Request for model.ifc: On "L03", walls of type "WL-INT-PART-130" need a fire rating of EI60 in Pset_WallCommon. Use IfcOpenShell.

First a look at what the model holds.

```python
import ifcopenshell
import ifcopenshell.util.element

model = ifcopenshell.open("model.ifc")
print(model.schema)
storey = next(s for s in model.by_type("IfcBuildingStorey") if s.Name == "L03")
walls = [e for e in ifcopenshell.util.element.get_decomposition(storey) if e.is_a("IfcWall")]
seen = {}
for e in walls:
    element_type = ifcopenshell.util.element.get_type(e)
    key = (element_type.Name if element_type != e and element_type else None, ifcopenshell.util.element.get_pset(e, "Pset_WallCommon", "FireRating"))
    seen[key] = seen.get(key, 0) + 1
for (name, value), count in sorted(seen.items(), key=str):
    print(count, "x", name, "|", value)
```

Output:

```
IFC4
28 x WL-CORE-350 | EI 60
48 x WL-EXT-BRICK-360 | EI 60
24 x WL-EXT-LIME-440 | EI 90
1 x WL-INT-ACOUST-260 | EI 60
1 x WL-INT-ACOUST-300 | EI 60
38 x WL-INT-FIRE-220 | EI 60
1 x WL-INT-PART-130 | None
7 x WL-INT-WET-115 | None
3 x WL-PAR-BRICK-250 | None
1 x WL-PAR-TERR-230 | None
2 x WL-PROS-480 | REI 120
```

```python
import ifcopenshell
import ifcopenshell.api.pset
import ifcopenshell.util.element

model = ifcopenshell.open("model.ifc")

storey = next(s for s in model.by_type("IfcBuildingStorey") if s.Name == "L03")
walls = [e for e in ifcopenshell.util.element.get_decomposition(storey) if e.is_a("IfcWall")]

count = 0
for e in walls:
    element_type = ifcopenshell.util.element.get_type(e)
    if element_type in (None, e) or element_type.Name != "WL-INT-PART-130":
        continue
    # add_pset returns the element's existing set when there is one.
    pset = ifcopenshell.api.pset.add_pset(model, product=e, name="Pset_WallCommon")
    ifcopenshell.api.pset.edit_pset(model, pset=pset, properties={"FireRating": "EI60"})
    count += 1

print(count, "walls updated")

model.write("model-out.ifc")
```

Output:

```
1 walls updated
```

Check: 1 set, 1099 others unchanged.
